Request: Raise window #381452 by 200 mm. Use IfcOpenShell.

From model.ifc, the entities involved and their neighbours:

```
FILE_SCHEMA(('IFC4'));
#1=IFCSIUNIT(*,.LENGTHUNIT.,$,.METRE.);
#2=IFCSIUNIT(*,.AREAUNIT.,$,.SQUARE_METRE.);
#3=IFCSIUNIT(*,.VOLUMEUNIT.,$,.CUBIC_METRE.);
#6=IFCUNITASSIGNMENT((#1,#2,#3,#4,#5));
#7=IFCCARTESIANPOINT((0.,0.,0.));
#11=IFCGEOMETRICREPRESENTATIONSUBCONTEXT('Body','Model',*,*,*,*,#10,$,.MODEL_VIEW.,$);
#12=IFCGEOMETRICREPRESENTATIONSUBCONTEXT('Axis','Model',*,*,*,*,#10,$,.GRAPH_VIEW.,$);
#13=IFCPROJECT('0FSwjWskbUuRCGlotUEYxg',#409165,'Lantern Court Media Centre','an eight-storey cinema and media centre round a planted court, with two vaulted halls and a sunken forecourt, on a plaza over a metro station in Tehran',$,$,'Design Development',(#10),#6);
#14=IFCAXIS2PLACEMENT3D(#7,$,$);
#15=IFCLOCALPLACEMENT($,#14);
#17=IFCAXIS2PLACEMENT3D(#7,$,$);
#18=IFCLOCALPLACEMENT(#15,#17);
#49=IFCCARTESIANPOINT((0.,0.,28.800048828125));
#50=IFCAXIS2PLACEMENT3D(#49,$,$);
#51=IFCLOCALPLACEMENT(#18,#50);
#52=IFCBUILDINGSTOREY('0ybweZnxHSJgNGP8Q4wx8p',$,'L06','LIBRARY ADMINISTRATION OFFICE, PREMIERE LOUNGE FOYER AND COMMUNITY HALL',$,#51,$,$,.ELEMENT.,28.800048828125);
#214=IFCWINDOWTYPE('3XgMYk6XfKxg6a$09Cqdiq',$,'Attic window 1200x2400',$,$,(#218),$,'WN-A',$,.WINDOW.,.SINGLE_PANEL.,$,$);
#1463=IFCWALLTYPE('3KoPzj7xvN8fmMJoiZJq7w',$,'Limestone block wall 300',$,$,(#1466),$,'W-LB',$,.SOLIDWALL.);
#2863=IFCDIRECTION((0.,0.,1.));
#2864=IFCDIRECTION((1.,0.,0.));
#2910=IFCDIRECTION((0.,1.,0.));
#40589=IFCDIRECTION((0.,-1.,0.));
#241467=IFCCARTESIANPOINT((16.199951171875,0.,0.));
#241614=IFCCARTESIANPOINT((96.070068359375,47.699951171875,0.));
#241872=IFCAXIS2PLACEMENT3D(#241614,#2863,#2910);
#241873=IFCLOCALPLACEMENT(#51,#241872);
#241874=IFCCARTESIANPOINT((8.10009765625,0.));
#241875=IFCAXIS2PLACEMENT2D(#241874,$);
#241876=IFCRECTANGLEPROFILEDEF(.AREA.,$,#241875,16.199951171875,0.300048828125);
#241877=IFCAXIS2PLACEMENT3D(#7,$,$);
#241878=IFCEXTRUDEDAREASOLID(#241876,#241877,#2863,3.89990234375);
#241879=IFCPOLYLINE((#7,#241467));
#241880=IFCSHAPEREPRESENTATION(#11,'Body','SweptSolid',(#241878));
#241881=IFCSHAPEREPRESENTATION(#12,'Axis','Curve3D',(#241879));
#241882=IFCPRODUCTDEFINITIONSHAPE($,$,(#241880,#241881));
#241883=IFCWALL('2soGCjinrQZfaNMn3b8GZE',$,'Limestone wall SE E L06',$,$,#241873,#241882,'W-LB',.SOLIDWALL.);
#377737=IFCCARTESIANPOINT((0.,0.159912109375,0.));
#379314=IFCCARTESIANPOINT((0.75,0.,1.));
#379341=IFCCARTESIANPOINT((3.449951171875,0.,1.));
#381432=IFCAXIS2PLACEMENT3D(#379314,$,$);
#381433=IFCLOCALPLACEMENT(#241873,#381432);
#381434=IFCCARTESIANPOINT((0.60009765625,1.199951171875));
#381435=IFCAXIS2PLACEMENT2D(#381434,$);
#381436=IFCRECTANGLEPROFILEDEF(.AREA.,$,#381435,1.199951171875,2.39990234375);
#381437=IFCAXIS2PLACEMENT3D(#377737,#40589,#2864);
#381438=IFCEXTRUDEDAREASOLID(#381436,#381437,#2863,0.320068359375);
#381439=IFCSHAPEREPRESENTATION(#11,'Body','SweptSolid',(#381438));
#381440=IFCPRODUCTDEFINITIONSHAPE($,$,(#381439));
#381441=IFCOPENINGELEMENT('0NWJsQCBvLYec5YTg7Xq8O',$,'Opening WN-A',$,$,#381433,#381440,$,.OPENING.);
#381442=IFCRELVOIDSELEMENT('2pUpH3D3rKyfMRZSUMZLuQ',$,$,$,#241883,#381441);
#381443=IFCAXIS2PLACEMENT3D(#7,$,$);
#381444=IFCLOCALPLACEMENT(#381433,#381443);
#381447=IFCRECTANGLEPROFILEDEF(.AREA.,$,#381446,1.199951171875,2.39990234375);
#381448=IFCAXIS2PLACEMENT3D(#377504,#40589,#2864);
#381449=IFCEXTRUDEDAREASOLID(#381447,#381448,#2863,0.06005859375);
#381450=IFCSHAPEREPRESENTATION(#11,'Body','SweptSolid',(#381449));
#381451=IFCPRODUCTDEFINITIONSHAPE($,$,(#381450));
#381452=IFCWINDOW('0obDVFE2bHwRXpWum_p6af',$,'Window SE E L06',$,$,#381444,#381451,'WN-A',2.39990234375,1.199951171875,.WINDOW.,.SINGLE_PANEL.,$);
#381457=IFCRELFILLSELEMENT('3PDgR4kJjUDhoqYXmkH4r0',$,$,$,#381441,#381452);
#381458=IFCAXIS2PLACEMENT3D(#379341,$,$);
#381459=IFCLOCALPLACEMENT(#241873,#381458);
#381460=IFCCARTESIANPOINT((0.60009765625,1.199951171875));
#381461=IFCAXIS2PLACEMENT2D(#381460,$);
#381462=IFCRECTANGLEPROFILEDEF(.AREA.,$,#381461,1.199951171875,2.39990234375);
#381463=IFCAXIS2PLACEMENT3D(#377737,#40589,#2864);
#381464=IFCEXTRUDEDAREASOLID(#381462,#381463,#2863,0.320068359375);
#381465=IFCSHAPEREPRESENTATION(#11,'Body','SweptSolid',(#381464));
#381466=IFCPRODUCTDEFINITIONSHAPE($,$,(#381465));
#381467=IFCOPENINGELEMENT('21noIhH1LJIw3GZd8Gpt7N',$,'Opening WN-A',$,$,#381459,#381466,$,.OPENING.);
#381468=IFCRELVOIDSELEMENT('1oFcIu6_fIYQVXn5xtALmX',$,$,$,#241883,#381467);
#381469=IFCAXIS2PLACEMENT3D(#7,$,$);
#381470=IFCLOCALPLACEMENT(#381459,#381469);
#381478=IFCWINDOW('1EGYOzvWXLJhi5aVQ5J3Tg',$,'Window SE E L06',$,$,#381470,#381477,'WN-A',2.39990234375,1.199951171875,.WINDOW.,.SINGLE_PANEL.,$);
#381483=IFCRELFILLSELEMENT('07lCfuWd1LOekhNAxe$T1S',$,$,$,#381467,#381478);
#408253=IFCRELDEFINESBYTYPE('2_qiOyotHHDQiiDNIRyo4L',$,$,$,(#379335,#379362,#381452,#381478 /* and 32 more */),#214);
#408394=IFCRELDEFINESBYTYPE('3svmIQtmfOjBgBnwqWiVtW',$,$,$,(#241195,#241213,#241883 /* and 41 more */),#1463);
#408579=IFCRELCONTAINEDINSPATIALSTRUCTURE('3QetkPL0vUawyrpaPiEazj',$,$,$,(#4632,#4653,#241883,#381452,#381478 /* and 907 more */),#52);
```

```python
import numpy as np
import ifcopenshell
import ifcopenshell.api.geometry
import ifcopenshell.util.placement
import ifcopenshell.util.unit

model = ifcopenshell.open("model.ifc")
unit_scale = ifcopenshell.util.unit.calculate_unit_scale(model)

window = model.by_guid("0obDVFE2bHwRXpWum_p6af")
opening = window.FillsVoids[0].RelatingOpeningElement
dz = 0.2 / unit_scale

shift = np.array([0.0, 0.0, dz])
# The window is placed relative to its opening, so it follows when the opening moves.
matrix = ifcopenshell.util.placement.get_local_placement(opening.ObjectPlacement)
matrix[:3, 3] += shift
ifcopenshell.api.geometry.edit_object_placement(
    model, product=opening, matrix=matrix, is_si=False, should_transform_children=True
)

print(f"moved by {dz * unit_scale:+.3f} m")

model.write("model_v2.ifc")
```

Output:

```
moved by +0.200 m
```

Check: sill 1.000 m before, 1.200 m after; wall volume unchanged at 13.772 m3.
